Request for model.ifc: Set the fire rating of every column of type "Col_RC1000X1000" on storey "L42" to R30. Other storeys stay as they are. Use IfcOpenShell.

First a look at what the model holds.

```python
import ifcopenshell
import ifcopenshell.util.element

model = ifcopenshell.open("model.ifc")
print(model.schema)
storey = next(s for s in model.by_type("IfcBuildingStorey") if s.Name == "L42")
columns = [e for e in ifcopenshell.util.element.get_decomposition(storey) if e.is_a("IfcColumn")]
seen = {}
for e in columns:
    element_type = ifcopenshell.util.element.get_type(e)
    key = (element_type.Name if element_type != e and element_type else None, ifcopenshell.util.element.get_pset(e, "Pset_ColumnCommon", "FireRating"))
    seen[key] = seen.get(key, 0) + 1
for (name, value), count in sorted(seen.items(), key=str):
    print(count, "x", name, "|", value)
```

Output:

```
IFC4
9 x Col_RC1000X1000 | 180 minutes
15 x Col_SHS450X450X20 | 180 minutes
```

```python
import ifcopenshell
import ifcopenshell.api.pset
import ifcopenshell.util.element

model = ifcopenshell.open("model.ifc")

storey = next(s for s in model.by_type("IfcBuildingStorey") if s.Name == "L42")
columns = [e for e in ifcopenshell.util.element.get_decomposition(storey) if e.is_a("IfcColumn")]

count = 0
for e in columns:
    element_type = ifcopenshell.util.element.get_type(e)
    if element_type in (None, e) or element_type.Name != "Col_RC1000X1000":
        continue
    # add_pset returns the element's existing set when there is one.
    pset = ifcopenshell.api.pset.add_pset(model, product=e, name="Pset_ColumnCommon")
    ifcopenshell.api.pset.edit_pset(model, pset=pset, properties={"FireRating": "R30"})
    count += 1

print(count, "columns updated")

model.write("model_updated.ifc")
```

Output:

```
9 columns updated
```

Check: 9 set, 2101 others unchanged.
